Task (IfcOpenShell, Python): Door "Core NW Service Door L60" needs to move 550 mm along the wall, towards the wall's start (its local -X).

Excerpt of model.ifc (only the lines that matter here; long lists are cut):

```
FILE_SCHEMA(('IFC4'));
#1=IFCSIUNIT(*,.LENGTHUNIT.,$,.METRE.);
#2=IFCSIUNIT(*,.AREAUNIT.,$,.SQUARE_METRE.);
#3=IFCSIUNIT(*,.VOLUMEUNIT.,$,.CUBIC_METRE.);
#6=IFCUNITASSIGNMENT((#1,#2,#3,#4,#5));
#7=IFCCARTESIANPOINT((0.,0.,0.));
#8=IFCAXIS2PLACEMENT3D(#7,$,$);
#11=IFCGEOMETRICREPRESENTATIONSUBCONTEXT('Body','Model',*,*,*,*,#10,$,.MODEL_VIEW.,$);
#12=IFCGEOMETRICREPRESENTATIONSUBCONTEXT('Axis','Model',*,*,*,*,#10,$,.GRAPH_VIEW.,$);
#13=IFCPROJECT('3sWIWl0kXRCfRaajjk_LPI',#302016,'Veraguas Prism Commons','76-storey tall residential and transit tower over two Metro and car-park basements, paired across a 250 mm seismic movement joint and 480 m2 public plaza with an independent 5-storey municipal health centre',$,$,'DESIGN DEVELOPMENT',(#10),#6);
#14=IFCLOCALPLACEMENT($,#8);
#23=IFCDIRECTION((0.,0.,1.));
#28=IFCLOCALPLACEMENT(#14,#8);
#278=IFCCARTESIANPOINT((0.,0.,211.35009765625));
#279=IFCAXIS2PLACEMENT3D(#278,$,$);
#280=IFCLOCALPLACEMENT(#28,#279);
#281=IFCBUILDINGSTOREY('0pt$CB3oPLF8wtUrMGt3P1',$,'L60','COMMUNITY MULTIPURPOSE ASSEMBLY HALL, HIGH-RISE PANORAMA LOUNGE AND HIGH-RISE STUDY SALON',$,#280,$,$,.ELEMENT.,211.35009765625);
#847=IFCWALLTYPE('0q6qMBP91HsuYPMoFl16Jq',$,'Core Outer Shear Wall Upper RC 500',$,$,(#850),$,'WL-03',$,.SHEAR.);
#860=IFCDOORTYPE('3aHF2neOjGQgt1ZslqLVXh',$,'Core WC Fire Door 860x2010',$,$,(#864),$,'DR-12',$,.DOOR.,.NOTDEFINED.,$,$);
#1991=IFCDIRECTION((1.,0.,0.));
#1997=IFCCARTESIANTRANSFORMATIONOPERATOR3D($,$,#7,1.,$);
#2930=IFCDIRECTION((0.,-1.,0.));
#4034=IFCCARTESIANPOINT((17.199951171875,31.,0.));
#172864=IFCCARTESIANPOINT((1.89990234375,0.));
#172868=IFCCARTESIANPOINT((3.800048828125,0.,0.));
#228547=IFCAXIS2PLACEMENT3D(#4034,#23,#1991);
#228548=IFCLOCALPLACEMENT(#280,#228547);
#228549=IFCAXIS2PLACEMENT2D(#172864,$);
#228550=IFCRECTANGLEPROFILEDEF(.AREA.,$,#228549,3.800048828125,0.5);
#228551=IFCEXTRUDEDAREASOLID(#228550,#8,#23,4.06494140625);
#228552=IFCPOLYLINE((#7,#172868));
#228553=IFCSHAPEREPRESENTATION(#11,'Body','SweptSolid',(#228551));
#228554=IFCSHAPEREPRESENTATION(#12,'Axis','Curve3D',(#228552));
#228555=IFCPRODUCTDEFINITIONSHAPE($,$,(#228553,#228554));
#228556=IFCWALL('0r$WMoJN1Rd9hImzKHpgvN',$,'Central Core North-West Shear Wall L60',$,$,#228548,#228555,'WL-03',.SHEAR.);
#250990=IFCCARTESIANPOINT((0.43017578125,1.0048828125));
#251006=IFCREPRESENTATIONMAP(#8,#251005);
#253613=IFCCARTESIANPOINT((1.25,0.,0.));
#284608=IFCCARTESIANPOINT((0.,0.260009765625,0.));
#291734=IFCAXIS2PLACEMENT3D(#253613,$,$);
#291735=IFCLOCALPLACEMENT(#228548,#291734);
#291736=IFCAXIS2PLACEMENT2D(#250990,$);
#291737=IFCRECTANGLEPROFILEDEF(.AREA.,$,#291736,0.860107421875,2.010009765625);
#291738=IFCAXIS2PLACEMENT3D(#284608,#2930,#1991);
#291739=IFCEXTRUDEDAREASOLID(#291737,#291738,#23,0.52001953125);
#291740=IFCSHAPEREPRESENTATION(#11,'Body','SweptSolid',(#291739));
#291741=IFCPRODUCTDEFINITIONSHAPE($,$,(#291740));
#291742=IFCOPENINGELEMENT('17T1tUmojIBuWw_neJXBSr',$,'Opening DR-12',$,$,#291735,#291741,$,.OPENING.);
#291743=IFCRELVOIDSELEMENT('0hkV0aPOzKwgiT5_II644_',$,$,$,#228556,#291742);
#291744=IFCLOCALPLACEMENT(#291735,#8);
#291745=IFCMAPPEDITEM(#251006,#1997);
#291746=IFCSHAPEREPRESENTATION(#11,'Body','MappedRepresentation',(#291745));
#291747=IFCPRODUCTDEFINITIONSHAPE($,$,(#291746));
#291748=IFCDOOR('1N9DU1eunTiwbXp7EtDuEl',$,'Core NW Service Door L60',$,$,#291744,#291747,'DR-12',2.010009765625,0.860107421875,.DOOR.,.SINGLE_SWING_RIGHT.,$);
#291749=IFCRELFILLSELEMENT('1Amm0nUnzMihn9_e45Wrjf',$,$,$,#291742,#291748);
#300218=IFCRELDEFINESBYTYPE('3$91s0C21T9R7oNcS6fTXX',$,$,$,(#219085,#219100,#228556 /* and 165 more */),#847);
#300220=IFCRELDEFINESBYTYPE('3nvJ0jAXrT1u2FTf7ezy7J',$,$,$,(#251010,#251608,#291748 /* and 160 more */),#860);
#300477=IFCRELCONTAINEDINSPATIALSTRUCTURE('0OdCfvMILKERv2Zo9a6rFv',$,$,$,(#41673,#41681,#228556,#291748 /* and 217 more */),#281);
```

```python
import ifcopenshell
import ifcopenshell.api.geometry
import ifcopenshell.util.placement
import ifcopenshell.util.unit

model = ifcopenshell.open("model.ifc")
unit_scale = ifcopenshell.util.unit.calculate_unit_scale(model)

door = model.by_id(291748)
opening = door.FillsVoids[0].RelatingOpeningElement
wall = opening.VoidsElements[0].RelatingBuildingElement

wall_matrix = ifcopenshell.util.placement.get_local_placement(wall.ObjectPlacement)
shift = wall_matrix[:3, 0] * -0.55 / unit_scale
before = ifcopenshell.util.placement.get_local_placement(door.ObjectPlacement)[:3, 3].copy()

# The door is placed relative to its opening, so it follows when the opening moves.
matrix = ifcopenshell.util.placement.get_local_placement(opening.ObjectPlacement)
matrix[:3, 3] += shift
ifcopenshell.api.geometry.edit_object_placement(
    model, product=opening, matrix=matrix, is_si=False, should_transform_children=True
)

after = ifcopenshell.util.placement.get_local_placement(door.ObjectPlacement)[:3, 3]
print("door moved by", (after - before).round(3) + 0.0)

model.write("model-out.ifc")
```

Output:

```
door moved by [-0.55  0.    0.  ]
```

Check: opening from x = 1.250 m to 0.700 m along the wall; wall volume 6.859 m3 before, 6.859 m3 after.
